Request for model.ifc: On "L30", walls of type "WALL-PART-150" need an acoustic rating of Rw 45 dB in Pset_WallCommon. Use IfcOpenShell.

First a look at what the model holds.

```python
import ifcopenshell
import ifcopenshell.util.element

model = ifcopenshell.open("model.ifc")
print(model.schema)
storey = next(s for s in model.by_type("IfcBuildingStorey") if s.Name == "L30")
walls = [e for e in ifcopenshell.util.element.get_decomposition(storey) if e.is_a("IfcWall")]
seen = {}
for e in walls:
    element_type = ifcopenshell.util.element.get_type(e)
    key = (element_type.Name if element_type != e and element_type else None, ifcopenshell.util.element.get_pset(e, "Pset_WallCommon", "AcousticRating"))
    seen[key] = seen.get(key, 0) + 1
for (name, value), count in sorted(seen.items(), key=str):
    print(count, "x", name, "|", value)
```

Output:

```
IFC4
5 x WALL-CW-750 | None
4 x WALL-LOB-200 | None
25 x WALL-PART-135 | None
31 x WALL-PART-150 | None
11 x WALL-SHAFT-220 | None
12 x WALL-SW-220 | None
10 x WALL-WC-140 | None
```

```python
import ifcopenshell
import ifcopenshell.api.pset
import ifcopenshell.util.element

model = ifcopenshell.open("model.ifc")

storey = next(s for s in model.by_type("IfcBuildingStorey") if s.Name == "L30")
walls = [e for e in ifcopenshell.util.element.get_decomposition(storey) if e.is_a("IfcWall")]

count = 0
for e in walls:
    element_type = ifcopenshell.util.element.get_type(e)
    if element_type in (None, e) or element_type.Name != "WALL-PART-150":
        continue
    found = ifcopenshell.util.element.get_pset(e, "Pset_WallCommon", should_inherit=False)
    if found:
        pset = model.by_id(found["id"])
        if len(ifcopenshell.util.element.get_elements_by_pset(pset)) > 1:
            pset = ifcopenshell.api.pset.unshare_pset(model, products=[e], pset=pset)[0]
    else:
        pset = ifcopenshell.api.pset.add_pset(model, product=e, name="Pset_WallCommon")
    ifcopenshell.api.pset.edit_pset(model, pset=pset, properties={"AcousticRating": "Rw 45 dB"})
    count += 1

print(count, "walls updated")

model.write("model_v2.ifc")
```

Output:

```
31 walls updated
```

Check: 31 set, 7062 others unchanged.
